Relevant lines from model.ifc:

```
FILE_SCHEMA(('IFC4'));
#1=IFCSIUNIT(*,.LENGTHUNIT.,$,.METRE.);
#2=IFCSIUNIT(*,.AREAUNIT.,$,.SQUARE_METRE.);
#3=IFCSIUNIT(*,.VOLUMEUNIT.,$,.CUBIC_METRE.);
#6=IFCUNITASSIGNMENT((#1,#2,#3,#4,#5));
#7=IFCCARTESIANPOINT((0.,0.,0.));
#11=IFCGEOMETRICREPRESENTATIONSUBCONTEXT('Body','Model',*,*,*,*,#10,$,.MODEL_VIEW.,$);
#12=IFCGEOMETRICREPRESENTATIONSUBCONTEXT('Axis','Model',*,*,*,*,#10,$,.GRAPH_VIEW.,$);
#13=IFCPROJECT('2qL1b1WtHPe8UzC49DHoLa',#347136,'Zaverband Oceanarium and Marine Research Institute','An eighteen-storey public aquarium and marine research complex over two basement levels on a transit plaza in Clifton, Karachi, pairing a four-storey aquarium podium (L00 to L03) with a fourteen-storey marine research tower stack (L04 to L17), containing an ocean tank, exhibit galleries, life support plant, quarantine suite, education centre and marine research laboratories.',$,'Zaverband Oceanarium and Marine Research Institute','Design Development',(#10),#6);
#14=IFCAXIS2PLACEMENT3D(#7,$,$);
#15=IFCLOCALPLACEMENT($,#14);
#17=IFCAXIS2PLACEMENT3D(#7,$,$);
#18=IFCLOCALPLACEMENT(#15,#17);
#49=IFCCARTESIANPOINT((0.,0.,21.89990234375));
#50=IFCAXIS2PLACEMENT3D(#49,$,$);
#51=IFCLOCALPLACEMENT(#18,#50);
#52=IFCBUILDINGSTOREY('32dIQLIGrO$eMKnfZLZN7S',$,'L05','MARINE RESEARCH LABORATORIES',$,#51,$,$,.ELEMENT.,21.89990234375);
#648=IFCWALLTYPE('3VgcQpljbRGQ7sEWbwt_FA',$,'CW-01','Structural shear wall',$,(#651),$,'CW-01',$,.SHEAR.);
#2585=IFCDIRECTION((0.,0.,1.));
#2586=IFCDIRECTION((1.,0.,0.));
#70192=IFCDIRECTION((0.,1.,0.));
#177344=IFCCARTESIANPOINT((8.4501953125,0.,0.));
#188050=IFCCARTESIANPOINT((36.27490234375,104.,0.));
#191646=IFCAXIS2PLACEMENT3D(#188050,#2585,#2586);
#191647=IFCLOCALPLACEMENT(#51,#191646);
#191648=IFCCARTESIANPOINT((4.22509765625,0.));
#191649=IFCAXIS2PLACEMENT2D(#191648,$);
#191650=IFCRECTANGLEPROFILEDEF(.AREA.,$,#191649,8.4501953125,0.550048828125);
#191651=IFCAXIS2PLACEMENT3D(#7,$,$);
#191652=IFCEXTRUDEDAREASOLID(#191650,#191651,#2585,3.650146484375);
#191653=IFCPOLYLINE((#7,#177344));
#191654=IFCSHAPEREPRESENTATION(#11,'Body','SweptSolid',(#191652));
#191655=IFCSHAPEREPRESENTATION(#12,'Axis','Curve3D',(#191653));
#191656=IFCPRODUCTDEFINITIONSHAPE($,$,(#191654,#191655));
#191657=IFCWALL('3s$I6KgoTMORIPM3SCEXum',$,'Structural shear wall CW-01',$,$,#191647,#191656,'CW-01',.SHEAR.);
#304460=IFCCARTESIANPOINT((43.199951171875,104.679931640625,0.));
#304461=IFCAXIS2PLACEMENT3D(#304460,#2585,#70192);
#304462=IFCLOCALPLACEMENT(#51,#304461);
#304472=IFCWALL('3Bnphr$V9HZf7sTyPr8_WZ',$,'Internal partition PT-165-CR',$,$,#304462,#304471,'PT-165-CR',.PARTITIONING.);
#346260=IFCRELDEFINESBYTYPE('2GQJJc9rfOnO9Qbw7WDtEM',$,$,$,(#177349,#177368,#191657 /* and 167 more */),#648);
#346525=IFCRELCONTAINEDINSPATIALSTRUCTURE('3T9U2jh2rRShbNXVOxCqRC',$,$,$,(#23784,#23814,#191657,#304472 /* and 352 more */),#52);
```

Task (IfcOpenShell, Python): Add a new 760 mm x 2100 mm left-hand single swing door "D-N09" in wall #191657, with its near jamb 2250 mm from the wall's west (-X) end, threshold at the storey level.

```python
import numpy as np
import ifcopenshell
import ifcopenshell.api.feature
import ifcopenshell.api.geometry
import ifcopenshell.api.root
import ifcopenshell.api.spatial
import ifcopenshell.geom
import ifcopenshell.util.element
import ifcopenshell.util.placement
import ifcopenshell.util.representation
import ifcopenshell.util.shape
import ifcopenshell.util.unit

model = ifcopenshell.open("model.ifc")
unit_scale = ifcopenshell.util.unit.calculate_unit_scale(model)
settings = ifcopenshell.geom.settings()


def volume(element):
    """Net volume in cubic metres, openings subtracted."""
    shape = ifcopenshell.geom.create_shape(settings, element)
    return ifcopenshell.util.shape.get_volume(shape.geometry)


wall = model.by_guid("3s$I6KgoTMORIPM3SCEXum")
storey = ifcopenshell.util.element.get_container(wall, ifc_class="IfcBuildingStorey")
context = ifcopenshell.util.representation.get_context(model, "Model", "Body", "MODEL_VIEW")
before = volume(wall)

width, height, from_end, sill = 0.76, 2.1, 2.25, 0.0  # metres

# The wall runs along its own X axis, and the end named is its -X end.
wall_shape = ifcopenshell.geom.create_shape(settings, wall)
x, y, z = ifcopenshell.util.shape.get_vertices(wall_shape.geometry).T
start = x.min() + from_end
face, thickness = float(y.min()), float(y.max() - y.min())
wall_matrix = ifcopenshell.util.placement.get_local_placement(wall.ObjectPlacement)
level = ifcopenshell.util.placement.get_local_placement(storey.ObjectPlacement)[2, 3]


def in_wall(x, y):
    """Placement at x, y metres in the wall's axes, at sill height."""
    matrix = wall_matrix.copy()
    matrix[:, 3] = wall_matrix @ np.array([x / unit_scale, y / unit_scale, 0.0, 1.0])
    matrix[2, 3] = level + sill / unit_scale
    return matrix


# Opening: a box that overshoots both wall faces by 50 mm.
opening = ifcopenshell.api.root.create_entity(model, ifc_class="IfcOpeningElement", predefined_type="OPENING")
box = ifcopenshell.api.geometry.add_wall_representation(
    model, context=context, length=width, height=height, thickness=thickness + 0.1
)
ifcopenshell.api.geometry.assign_representation(model, product=opening, representation=box)
ifcopenshell.api.geometry.edit_object_placement(model, product=opening, matrix=in_wall(start, face - 0.05), is_si=False)
ifcopenshell.api.feature.add_feature(model, feature=opening, element=wall)

door = ifcopenshell.api.root.create_entity(model, ifc_class="IfcDoor", name="D-N09", predefined_type="DOOR")
door.OverallWidth, door.OverallHeight = width / unit_scale, height / unit_scale
door.OperationType = "SINGLE_SWING_LEFT"
body = ifcopenshell.api.geometry.add_door_representation(
    model,
    context=context,
    overall_width=door.OverallWidth,
    overall_height=door.OverallHeight,
    operation_type="SINGLE_SWING_LEFT",
    lining_properties={"LiningDepth": thickness / unit_scale, "ThresholdDepth": thickness / unit_scale},
)
ifcopenshell.api.geometry.assign_representation(model, product=door, representation=body)
ifcopenshell.api.spatial.assign_container(model, products=[door], relating_structure=storey)
ifcopenshell.api.feature.add_filling(model, opening=opening, element=door)

# The lining spans the wall, so the door starts at the wall face.
ifcopenshell.api.geometry.edit_object_placement(model, product=door, matrix=in_wall(start, face), is_si=False)

after = volume(wall)

print(f"wall volume {before:.3f} -> {after:.3f} m3")

model.write("model-out.ifc")
```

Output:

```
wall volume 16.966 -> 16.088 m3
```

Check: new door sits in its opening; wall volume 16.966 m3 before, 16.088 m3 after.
